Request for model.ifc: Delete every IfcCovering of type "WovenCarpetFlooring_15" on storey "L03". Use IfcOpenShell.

First a look at what the model holds.

```python
import ifcopenshell
import ifcopenshell.util.element

model = ifcopenshell.open("model.ifc")
print(model.schema)
storey = next(s for s in model.by_type("IfcBuildingStorey") if s.Name == "L03")
coverings = [e for e in ifcopenshell.util.element.get_decomposition(storey) if e.is_a("IfcCovering")]
seen = {}
for e in coverings:
    element_type = ifcopenshell.util.element.get_type(e)
    name = element_type.Name if element_type not in (None, e) else None
    seen[name] = seen.get(name, 0) + 1
for name, count in sorted(seen.items(), key=str):
    print(count, "x", name)
```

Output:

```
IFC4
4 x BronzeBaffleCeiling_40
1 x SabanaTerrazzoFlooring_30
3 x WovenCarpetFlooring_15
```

```python
import ifcopenshell
import ifcopenshell.api.root
import ifcopenshell.util.element

model = ifcopenshell.open("model.ifc")

storey = next(s for s in model.by_type("IfcBuildingStorey") if s.Name == "L03")
coverings = [e for e in ifcopenshell.util.element.get_decomposition(storey) if e.is_a("IfcCovering")]
targets = [e for e in coverings if (t := ifcopenshell.util.element.get_type(e)) not in (None, e) and t.Name == "WovenCarpetFlooring_15"]

for e in targets:
    ifcopenshell.api.root.remove_product(model, product=e)
print(len(targets), "removed")

model.write("model_v2.ifc")
```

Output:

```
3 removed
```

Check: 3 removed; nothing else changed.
